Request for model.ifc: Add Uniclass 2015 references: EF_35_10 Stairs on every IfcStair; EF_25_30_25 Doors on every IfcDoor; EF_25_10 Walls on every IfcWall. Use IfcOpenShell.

First a look at what the model holds.

```python
import ifcopenshell

model = ifcopenshell.open("model.ifc")
print(model.schema)
print("classifications:", [c.Name for c in model.by_type("IfcClassification")])
for ifc_class in ("IfcDoor", "IfcRoof", "IfcStair", "IfcWall", "IfcWindow"):
    print(ifc_class, len(model.by_type(ifc_class)))
```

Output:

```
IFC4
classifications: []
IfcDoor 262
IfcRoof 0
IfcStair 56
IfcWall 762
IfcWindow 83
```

```python
import ifcopenshell
import ifcopenshell.api.classification

model = ifcopenshell.open("model.ifc")

system = ifcopenshell.api.classification.add_classification(model, classification="Uniclass 2015")

codes = {
    "IfcStair": ("EF_35_10", "Stairs"),
    "IfcDoor": ("EF_25_30_25", "Doors"),
    "IfcWall": ("EF_25_10", "Walls"),
}
for ifc_class, (code, name) in codes.items():
    products = model.by_type(ifc_class)
    ifcopenshell.api.classification.add_reference(
        model, products=products, classification=system, identification=code, name=name
    )
    print(code, len(products))

model.write("model_edited.ifc")
```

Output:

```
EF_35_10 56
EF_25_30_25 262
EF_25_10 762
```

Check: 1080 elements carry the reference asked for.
